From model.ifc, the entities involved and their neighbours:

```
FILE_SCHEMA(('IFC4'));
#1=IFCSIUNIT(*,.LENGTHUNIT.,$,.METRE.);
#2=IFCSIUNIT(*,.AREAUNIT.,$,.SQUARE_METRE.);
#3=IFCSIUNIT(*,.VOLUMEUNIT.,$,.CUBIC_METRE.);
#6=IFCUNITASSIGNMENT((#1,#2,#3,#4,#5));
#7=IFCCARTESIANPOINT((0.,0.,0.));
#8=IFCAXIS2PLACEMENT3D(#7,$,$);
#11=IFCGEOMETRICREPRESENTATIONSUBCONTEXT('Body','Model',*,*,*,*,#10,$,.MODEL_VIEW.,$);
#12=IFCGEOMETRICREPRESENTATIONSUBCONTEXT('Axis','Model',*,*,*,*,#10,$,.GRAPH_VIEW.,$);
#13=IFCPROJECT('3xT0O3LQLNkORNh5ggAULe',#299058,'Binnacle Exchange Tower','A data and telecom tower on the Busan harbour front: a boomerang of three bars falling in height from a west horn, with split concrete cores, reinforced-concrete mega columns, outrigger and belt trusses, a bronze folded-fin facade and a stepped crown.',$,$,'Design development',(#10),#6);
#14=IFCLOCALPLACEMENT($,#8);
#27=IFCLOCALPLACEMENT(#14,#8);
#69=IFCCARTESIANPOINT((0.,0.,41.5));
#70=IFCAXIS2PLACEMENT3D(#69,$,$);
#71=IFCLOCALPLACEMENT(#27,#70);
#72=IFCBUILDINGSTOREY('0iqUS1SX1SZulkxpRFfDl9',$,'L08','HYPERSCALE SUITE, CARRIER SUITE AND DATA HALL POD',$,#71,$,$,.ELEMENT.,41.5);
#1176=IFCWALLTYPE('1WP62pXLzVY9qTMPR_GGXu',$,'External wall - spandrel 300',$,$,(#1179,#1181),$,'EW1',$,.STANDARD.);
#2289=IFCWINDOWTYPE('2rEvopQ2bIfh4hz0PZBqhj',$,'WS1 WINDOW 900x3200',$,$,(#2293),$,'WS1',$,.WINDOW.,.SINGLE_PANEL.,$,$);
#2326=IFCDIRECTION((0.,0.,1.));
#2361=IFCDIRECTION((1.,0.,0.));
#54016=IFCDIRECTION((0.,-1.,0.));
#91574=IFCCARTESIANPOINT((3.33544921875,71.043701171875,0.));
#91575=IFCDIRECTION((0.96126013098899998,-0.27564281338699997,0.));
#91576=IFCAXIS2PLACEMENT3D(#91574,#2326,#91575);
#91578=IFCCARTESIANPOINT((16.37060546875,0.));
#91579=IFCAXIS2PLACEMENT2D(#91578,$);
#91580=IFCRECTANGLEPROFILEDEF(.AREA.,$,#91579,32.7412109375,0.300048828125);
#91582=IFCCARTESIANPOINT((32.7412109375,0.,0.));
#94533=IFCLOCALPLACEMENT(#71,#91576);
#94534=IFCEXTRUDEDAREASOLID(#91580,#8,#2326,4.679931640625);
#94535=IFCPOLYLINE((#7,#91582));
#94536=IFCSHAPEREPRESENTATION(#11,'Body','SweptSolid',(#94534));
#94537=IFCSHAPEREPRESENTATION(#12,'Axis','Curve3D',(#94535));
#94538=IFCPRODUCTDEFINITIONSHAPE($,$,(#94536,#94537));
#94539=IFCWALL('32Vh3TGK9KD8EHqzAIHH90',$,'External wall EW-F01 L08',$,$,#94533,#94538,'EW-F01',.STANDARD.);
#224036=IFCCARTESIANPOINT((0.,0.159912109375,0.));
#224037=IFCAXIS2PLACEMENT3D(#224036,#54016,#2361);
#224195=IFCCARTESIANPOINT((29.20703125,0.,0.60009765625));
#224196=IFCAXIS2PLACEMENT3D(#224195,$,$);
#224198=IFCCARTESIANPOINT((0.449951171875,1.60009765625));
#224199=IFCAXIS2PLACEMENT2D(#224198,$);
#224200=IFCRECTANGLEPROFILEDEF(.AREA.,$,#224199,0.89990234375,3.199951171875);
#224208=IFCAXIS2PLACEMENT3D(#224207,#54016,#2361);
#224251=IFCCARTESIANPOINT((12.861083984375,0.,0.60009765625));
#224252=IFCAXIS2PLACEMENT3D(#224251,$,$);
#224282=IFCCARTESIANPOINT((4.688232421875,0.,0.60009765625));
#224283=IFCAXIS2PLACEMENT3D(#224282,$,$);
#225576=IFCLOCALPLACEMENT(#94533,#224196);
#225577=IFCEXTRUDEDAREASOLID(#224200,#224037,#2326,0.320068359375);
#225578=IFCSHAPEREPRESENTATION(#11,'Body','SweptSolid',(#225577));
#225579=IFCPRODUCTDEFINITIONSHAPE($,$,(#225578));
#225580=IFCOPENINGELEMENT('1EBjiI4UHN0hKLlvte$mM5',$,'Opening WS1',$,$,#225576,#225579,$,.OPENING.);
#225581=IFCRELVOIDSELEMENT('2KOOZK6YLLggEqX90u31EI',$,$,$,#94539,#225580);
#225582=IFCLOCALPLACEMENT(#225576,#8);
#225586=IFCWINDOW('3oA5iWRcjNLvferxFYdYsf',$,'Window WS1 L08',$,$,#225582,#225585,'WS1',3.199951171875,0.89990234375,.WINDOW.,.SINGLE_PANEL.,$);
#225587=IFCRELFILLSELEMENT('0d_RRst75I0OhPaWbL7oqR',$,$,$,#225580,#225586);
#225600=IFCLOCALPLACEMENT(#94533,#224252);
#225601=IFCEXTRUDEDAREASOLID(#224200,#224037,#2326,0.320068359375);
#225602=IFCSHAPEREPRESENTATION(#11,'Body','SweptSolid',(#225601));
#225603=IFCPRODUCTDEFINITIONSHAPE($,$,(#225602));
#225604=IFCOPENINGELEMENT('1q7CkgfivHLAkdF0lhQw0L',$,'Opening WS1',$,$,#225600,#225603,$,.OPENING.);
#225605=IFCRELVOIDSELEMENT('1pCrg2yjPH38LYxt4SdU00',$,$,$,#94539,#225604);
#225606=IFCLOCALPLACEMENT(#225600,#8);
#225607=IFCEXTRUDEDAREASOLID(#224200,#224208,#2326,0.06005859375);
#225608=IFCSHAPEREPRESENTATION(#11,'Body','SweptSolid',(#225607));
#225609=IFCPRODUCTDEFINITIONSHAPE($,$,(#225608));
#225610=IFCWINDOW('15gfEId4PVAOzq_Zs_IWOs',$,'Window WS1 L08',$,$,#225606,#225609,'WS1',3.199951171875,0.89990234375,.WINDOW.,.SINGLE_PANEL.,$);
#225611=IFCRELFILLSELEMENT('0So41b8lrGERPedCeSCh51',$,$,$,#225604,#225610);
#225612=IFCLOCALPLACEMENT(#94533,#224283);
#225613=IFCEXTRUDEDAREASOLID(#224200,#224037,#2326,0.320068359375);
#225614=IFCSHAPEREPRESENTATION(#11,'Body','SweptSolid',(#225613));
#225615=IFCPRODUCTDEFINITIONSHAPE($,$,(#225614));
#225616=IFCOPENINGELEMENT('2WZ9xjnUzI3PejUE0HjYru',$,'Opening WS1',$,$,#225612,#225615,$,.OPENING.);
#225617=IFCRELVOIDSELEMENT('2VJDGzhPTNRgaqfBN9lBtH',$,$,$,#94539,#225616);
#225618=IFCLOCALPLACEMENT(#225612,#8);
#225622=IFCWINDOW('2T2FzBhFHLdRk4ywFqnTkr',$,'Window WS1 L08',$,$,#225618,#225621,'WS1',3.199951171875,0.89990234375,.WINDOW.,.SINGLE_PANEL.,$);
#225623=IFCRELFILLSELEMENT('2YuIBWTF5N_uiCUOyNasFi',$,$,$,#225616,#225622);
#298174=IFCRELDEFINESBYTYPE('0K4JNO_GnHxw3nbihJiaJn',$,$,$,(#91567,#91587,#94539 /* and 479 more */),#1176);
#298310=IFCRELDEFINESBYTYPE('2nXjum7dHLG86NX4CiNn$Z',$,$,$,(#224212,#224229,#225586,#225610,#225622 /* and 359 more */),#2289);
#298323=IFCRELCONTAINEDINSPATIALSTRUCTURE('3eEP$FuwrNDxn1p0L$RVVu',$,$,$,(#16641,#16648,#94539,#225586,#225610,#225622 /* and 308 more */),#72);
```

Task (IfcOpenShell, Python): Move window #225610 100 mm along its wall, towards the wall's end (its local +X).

```python
import ifcopenshell
import ifcopenshell.api.geometry
import ifcopenshell.util.placement
import ifcopenshell.util.unit

model = ifcopenshell.open("model.ifc")
unit_scale = ifcopenshell.util.unit.calculate_unit_scale(model)

window = model.by_id(225610)
opening = window.FillsVoids[0].RelatingOpeningElement
wall = opening.VoidsElements[0].RelatingBuildingElement

wall_matrix = ifcopenshell.util.placement.get_local_placement(wall.ObjectPlacement)
shift = wall_matrix[:3, 0] * 0.1 / unit_scale
before = ifcopenshell.util.placement.get_local_placement(window.ObjectPlacement)[:3, 3].copy()

# The window is placed relative to its opening, so it follows when the opening moves.
matrix = ifcopenshell.util.placement.get_local_placement(opening.ObjectPlacement)
matrix[:3, 3] += shift
ifcopenshell.api.geometry.edit_object_placement(
    model, product=opening, matrix=matrix, is_si=False, should_transform_children=True
)

after = ifcopenshell.util.placement.get_local_placement(window.ObjectPlacement)[:3, 3]
print("window moved by", (after - before).round(3) + 0.0)

model.write("model-out.ifc")
```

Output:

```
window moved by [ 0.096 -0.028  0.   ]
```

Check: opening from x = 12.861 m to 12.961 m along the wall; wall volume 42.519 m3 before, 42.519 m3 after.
